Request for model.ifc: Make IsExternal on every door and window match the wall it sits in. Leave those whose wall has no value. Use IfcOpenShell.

First a look at what the model holds.

```python
import ifcopenshell
import ifcopenshell.util.element

model = ifcopenshell.open("model.ifc")
print(model.schema)
seen = {}
for e in model.by_type("IfcDoor") + model.by_type("IfcWindow"):
    if not e.FillsVoids:
        continue
    host = e.FillsVoids[0].RelatingOpeningElement.VoidsElements[0].RelatingBuildingElement
    own = ifcopenshell.util.element.get_pset(e, f"Pset_{e.is_a()[3:].removesuffix('StandardCase')}Common", "IsExternal")
    wall = ifcopenshell.util.element.get_pset(host, "Pset_WallCommon", "IsExternal")
    seen[e.is_a(), own, wall] = seen.get((e.is_a(), own, wall), 0) + 1
for (cls, own, wall), count in sorted(seen.items(), key=str):
    print(count, cls, "IsExternal:", own, "| host wall:", wall)
```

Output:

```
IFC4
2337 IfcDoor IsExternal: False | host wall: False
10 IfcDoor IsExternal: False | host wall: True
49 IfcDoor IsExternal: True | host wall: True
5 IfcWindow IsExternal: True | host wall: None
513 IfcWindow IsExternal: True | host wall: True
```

```python
import ifcopenshell
import ifcopenshell.api.pset
import ifcopenshell.util.element

model = ifcopenshell.open("model.ifc")

count = 0
for ifc_class, pset_name in (("IfcDoor", "Pset_DoorCommon"), ("IfcWindow", "Pset_WindowCommon")):
    for e in model.by_type(ifc_class):
        if not e.FillsVoids:
            continue
        host = e.FillsVoids[0].RelatingOpeningElement.VoidsElements[0].RelatingBuildingElement
        external = ifcopenshell.util.element.get_pset(host, "Pset_WallCommon", "IsExternal")
        if external is None or ifcopenshell.util.element.get_pset(e, pset_name, "IsExternal") == external:
            continue
        found = ifcopenshell.util.element.get_pset(e, pset_name, should_inherit=False)
        if found:
            pset = model.by_id(found["id"])
            if len(ifcopenshell.util.element.get_elements_by_pset(pset)) > 1:
                pset = ifcopenshell.api.pset.unshare_pset(model, products=[e], pset=pset)[0]
        else:
            pset = ifcopenshell.api.pset.add_pset(model, product=e, name=pset_name)
        ifcopenshell.api.pset.edit_pset(model, pset=pset, properties={"IsExternal": external})
        count += 1

print(count, "updated")

model.write("model_edited.ifc")
```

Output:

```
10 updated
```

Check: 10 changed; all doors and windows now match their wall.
